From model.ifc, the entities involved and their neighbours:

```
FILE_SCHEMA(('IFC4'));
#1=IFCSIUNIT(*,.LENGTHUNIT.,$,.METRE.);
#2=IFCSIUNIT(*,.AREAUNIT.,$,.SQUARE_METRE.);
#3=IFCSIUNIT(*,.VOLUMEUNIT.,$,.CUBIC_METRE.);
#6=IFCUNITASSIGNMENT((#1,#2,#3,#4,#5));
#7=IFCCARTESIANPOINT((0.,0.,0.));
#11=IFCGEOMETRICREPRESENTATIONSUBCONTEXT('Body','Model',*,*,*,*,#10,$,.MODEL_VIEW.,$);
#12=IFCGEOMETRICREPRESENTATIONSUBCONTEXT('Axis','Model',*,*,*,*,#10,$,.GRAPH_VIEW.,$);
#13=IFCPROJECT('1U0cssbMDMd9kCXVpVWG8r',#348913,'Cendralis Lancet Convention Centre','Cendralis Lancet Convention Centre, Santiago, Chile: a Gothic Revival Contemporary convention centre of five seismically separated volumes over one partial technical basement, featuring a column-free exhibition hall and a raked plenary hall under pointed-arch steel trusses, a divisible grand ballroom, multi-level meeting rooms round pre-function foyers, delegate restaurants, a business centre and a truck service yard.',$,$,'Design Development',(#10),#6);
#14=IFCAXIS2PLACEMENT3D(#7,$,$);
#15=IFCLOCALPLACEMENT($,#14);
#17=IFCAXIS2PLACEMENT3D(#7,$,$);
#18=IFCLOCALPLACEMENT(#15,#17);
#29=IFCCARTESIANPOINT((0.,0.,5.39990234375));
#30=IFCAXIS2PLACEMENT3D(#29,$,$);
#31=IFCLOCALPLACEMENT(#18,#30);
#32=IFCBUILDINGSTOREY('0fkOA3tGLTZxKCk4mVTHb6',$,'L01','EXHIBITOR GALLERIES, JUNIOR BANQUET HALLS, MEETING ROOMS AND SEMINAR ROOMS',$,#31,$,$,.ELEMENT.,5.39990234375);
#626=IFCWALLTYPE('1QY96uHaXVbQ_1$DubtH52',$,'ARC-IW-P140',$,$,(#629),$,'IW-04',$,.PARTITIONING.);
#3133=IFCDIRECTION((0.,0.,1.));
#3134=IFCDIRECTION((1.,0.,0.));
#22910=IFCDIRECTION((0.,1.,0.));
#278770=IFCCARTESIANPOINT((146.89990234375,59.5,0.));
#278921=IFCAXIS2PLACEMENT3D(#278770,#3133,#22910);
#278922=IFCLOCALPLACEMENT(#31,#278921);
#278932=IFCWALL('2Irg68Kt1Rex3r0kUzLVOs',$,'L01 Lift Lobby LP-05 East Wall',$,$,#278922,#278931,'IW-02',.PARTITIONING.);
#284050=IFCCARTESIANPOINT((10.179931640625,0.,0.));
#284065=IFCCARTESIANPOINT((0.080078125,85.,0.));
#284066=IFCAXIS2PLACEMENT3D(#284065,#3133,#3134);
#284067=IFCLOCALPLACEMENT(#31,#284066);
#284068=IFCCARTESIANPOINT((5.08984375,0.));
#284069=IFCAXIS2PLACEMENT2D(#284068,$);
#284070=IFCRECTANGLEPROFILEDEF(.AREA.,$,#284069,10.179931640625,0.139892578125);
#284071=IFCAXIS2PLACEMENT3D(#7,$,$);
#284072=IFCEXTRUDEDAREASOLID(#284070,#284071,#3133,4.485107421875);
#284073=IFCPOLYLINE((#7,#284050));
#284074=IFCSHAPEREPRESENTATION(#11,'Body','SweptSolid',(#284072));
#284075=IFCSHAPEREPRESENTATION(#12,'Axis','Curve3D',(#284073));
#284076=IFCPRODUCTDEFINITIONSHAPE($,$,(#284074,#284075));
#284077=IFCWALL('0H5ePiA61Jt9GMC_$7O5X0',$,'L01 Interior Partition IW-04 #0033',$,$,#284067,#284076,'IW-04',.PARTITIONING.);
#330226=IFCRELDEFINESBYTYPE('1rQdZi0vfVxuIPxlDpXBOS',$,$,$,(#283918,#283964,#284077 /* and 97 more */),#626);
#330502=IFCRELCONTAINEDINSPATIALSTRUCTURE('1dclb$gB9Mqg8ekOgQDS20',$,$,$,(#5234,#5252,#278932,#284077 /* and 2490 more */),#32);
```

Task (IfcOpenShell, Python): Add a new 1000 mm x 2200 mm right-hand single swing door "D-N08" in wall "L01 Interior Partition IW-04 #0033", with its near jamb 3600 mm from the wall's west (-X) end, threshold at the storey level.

```python
import numpy as np
import ifcopenshell
import ifcopenshell.api.feature
import ifcopenshell.api.geometry
import ifcopenshell.api.root
import ifcopenshell.api.spatial
import ifcopenshell.geom
import ifcopenshell.util.element
import ifcopenshell.util.placement
import ifcopenshell.util.representation
import ifcopenshell.util.shape
import ifcopenshell.util.unit

model = ifcopenshell.open("model.ifc")
unit_scale = ifcopenshell.util.unit.calculate_unit_scale(model)
settings = ifcopenshell.geom.settings()


def volume(element):
    """Net volume in cubic metres, openings subtracted."""
    shape = ifcopenshell.geom.create_shape(settings, element)
    return ifcopenshell.util.shape.get_volume(shape.geometry)


wall = model.by_guid("0H5ePiA61Jt9GMC_$7O5X0")
storey = ifcopenshell.util.element.get_container(wall, ifc_class="IfcBuildingStorey")
context = ifcopenshell.util.representation.get_context(model, "Model", "Body", "MODEL_VIEW")
before = volume(wall)

width, height, from_end, sill = 1, 2.2, 3.6, 0.0  # metres

# The wall runs along its own X axis, and the end named is its -X end.
wall_shape = ifcopenshell.geom.create_shape(settings, wall)
x, y, z = ifcopenshell.util.shape.get_vertices(wall_shape.geometry).T
start = x.min() + from_end
face, thickness = float(y.min()), float(y.max() - y.min())
wall_matrix = ifcopenshell.util.placement.get_local_placement(wall.ObjectPlacement)
level = ifcopenshell.util.placement.get_local_placement(storey.ObjectPlacement)[2, 3]


def in_wall(x, y):
    """Placement at x, y metres in the wall's axes, at sill height."""
    matrix = wall_matrix.copy()
    matrix[:, 3] = wall_matrix @ np.array([x / unit_scale, y / unit_scale, 0.0, 1.0])
    matrix[2, 3] = level + sill / unit_scale
    return matrix


# Opening: a box that overshoots both wall faces by 50 mm.
opening = ifcopenshell.api.root.create_entity(model, ifc_class="IfcOpeningElement", predefined_type="OPENING")
box = ifcopenshell.api.geometry.add_wall_representation(
    model, context=context, length=width, height=height, thickness=thickness + 0.1
)
ifcopenshell.api.geometry.assign_representation(model, product=opening, representation=box)
ifcopenshell.api.geometry.edit_object_placement(model, product=opening, matrix=in_wall(start, face - 0.05), is_si=False)
ifcopenshell.api.feature.add_feature(model, feature=opening, element=wall)

door = ifcopenshell.api.root.create_entity(model, ifc_class="IfcDoor", name="D-N08", predefined_type="DOOR")
door.OverallWidth, door.OverallHeight = width / unit_scale, height / unit_scale
door.OperationType = "SINGLE_SWING_RIGHT"
body = ifcopenshell.api.geometry.add_door_representation(
    model,
    context=context,
    overall_width=door.OverallWidth,
    overall_height=door.OverallHeight,
    operation_type="SINGLE_SWING_RIGHT",
    lining_properties={"LiningDepth": thickness / unit_scale, "ThresholdDepth": thickness / unit_scale},
)
ifcopenshell.api.geometry.assign_representation(model, product=door, representation=body)
ifcopenshell.api.spatial.assign_container(model, products=[door], relating_structure=storey)
ifcopenshell.api.feature.add_filling(model, opening=opening, element=door)

# The lining spans the wall, so the door starts at the wall face.
ifcopenshell.api.geometry.edit_object_placement(model, product=door, matrix=in_wall(start, face), is_si=False)

after = volume(wall)

print(f"wall volume {before:.3f} -> {after:.3f} m3")

model.write("model_edited.ifc")
```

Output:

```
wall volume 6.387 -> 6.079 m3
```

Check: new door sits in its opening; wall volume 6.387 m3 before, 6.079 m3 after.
